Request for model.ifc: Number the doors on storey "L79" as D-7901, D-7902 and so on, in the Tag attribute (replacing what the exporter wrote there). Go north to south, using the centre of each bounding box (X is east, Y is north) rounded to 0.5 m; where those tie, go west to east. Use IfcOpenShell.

First a look at what the model holds.

```python
import ifcopenshell
import ifcopenshell.util.element
import ifcopenshell.util.placement

model = ifcopenshell.open("model.ifc")
print(model.schema)
storey = next(s for s in model.by_type("IfcBuildingStorey") if s.Name == "L79")
doors = [e for e in ifcopenshell.util.element.get_decomposition(storey) if e.is_a("IfcDoor")]
for e in sorted(doors, key=lambda e: e.id()):
    origin = ifcopenshell.util.placement.get_local_placement(e.ObjectPlacement)[:3, 3]
    print(e.id(), e.Tag, e.Name, origin.round(2) + 0.0, sep=" | ")
```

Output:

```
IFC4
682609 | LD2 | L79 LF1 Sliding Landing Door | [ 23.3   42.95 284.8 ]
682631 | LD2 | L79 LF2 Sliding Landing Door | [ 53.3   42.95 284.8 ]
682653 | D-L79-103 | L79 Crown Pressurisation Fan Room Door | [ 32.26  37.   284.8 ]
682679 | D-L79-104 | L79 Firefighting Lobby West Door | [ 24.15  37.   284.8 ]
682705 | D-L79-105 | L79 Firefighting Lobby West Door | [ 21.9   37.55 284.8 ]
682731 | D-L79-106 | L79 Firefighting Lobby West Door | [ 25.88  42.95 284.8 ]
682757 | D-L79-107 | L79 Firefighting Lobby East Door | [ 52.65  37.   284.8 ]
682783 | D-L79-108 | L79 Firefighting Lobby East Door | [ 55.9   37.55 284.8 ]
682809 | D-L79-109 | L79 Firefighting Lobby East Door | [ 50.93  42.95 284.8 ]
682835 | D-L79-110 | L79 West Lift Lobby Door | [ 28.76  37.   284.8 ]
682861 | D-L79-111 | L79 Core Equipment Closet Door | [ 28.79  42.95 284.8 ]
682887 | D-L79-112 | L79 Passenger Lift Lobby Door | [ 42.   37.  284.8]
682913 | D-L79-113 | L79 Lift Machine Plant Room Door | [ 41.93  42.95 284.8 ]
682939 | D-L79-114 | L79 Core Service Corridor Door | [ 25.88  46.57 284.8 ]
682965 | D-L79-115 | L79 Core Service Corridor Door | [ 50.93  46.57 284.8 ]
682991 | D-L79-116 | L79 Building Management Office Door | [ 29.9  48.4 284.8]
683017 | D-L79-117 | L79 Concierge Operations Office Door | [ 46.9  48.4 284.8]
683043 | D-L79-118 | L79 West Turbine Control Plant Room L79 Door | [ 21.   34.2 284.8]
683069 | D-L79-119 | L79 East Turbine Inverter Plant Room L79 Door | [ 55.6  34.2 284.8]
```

```python
import ifcopenshell
import ifcopenshell.geom
import ifcopenshell.util.element
import ifcopenshell.util.shape

model = ifcopenshell.open("model.ifc")
settings = ifcopenshell.geom.settings()
settings.set("use-world-coords", True)


def centre(element):
    shape = ifcopenshell.geom.create_shape(settings, element)
    return ifcopenshell.util.shape.get_bbox_centroid(shape.geometry)


storey = next(s for s in model.by_type("IfcBuildingStorey") if s.Name == "L79")
doors = [e for e in ifcopenshell.util.element.get_decomposition(storey) if e.is_a("IfcDoor")]

# Insertion points can sit at a corner or the storey origin, so sort by the geometry (in metres).
centres = {e: centre(e) for e in doors}
doors.sort(key=lambda e: (-round(centres[e][1] / 0.5), centres[e][0]))

for i, e in enumerate(doors, start=1):
    number = f"D-79{i:02d}"
    e.Tag = number
    print(e.id(), number)

model.write("model_rev.ifc")
```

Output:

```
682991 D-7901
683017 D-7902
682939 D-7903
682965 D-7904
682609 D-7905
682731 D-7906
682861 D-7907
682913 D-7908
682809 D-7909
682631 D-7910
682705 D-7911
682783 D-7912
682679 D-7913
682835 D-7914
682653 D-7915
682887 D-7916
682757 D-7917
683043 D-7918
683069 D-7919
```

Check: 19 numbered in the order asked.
